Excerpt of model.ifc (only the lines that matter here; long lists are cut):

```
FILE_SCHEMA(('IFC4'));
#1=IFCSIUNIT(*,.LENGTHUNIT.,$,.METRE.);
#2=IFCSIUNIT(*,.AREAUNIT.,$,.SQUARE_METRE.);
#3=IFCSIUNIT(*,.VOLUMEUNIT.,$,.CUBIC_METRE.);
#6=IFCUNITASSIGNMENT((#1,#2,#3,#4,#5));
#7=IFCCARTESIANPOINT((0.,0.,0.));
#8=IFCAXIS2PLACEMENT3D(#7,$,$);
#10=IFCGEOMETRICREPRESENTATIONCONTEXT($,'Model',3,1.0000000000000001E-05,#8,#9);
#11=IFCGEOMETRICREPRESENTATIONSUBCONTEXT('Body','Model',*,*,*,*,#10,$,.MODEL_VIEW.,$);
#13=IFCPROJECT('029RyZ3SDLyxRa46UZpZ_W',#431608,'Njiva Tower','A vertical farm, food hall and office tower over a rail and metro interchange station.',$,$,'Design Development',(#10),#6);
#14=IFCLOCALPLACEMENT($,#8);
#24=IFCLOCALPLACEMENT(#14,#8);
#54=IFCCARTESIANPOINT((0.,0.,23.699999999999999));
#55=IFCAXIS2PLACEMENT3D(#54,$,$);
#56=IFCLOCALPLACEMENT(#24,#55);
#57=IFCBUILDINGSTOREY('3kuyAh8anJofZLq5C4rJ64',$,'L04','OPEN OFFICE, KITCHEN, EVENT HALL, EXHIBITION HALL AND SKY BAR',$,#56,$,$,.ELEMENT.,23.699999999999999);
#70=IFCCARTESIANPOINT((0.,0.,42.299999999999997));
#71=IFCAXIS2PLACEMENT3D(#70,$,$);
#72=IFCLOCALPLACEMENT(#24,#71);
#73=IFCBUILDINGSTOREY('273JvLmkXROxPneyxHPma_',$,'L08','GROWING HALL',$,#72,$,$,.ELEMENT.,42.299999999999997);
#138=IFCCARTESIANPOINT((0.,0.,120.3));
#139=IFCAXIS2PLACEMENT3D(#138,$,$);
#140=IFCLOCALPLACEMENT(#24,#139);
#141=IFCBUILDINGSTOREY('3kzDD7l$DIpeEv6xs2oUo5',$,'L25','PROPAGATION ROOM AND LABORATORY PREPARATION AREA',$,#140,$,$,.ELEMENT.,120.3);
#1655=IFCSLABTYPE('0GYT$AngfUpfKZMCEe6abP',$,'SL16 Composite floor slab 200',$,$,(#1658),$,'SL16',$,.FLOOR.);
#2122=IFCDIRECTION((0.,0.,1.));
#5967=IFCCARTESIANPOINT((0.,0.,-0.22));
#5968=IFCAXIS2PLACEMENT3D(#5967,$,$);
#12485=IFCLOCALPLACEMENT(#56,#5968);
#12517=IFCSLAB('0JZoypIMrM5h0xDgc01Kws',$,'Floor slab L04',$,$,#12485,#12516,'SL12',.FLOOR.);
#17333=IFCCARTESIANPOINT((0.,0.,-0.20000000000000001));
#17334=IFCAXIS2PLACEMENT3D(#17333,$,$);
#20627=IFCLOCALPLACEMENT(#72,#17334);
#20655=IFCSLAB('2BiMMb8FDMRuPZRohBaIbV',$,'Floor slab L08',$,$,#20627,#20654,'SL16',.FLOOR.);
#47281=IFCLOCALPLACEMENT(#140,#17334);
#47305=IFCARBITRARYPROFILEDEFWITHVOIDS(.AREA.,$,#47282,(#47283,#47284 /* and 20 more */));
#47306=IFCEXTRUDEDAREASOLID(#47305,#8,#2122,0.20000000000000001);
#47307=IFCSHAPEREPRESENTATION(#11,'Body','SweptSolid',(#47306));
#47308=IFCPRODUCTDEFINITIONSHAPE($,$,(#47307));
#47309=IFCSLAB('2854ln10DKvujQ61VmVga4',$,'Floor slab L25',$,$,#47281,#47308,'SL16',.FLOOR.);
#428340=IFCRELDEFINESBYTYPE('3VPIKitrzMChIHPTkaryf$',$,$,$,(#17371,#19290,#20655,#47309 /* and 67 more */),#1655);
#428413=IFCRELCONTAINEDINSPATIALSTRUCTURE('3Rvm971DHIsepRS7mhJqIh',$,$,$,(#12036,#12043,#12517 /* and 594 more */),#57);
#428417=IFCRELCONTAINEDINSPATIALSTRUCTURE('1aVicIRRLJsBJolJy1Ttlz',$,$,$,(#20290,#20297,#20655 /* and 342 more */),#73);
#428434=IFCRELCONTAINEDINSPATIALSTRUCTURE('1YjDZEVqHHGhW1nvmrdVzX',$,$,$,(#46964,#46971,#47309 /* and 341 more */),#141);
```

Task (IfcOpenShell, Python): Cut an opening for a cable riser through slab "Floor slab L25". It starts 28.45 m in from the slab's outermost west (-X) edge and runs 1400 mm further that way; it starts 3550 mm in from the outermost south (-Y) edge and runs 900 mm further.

```python
import numpy as np
import ifcopenshell
import ifcopenshell.api.feature
import ifcopenshell.api.geometry
import ifcopenshell.api.root
import ifcopenshell.geom
import ifcopenshell.util.placement
import ifcopenshell.util.representation
import ifcopenshell.util.shape
import ifcopenshell.util.unit

model = ifcopenshell.open("model.ifc")
unit_scale = ifcopenshell.util.unit.calculate_unit_scale(model)
settings = ifcopenshell.geom.settings()


def volume(element):
    """Net volume in cubic metres, openings subtracted."""
    shape = ifcopenshell.geom.create_shape(settings, element)
    return ifcopenshell.util.shape.get_volume(shape.geometry)


slab = model.by_guid("2854ln10DKvujQ61VmVga4")
before = volume(slab)

# Extent in the slab's own axes, in metres. The edges named are its -X and -Y sides.
slab_shape = ifcopenshell.geom.create_shape(settings, slab)
vertices = ifcopenshell.util.shape.get_vertices(slab_shape.geometry)
x_min, y_min, bottom = vertices.min(axis=0)
top = vertices[:, 2].max()

opening = ifcopenshell.api.root.create_entity(model, ifc_class="IfcOpeningElement", name="Cable riser opening", predefined_type="OPENING")
context = ifcopenshell.util.representation.get_context(model, "Model", "Body", "MODEL_VIEW")
width, depth = 1.4, 0.9
outline = [(0.0, 0.0), (width, 0.0), (width, depth), (0.0, depth), (0.0, 0.0)]
# Overshoot both faces by 50 mm so the cut is clean.
shape = ifcopenshell.api.geometry.add_slab_representation(
    model, context=context, depth=top - bottom + 0.1, polyline=outline
)
ifcopenshell.api.geometry.assign_representation(model, product=opening, representation=shape)

matrix = ifcopenshell.util.placement.get_local_placement(slab.ObjectPlacement)
matrix[:, 3] = matrix @ np.append(np.array([x_min + 28.45, y_min + 3.55, bottom - 0.05]) / unit_scale, 1.0)
ifcopenshell.api.geometry.edit_object_placement(model, product=opening, matrix=matrix, is_si=False)
ifcopenshell.api.feature.add_feature(model, feature=opening, element=slab)

after = volume(slab)

print(f"slab volume {before:.3f} -> {after:.3f} m3")

model.write("model-out.ifc")
```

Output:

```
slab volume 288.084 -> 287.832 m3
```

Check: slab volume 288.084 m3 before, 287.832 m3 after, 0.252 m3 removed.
